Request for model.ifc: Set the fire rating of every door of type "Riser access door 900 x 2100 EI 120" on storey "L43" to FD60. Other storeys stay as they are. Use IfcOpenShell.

First a look at what the model holds.

```python
import ifcopenshell
import ifcopenshell.util.element

model = ifcopenshell.open("model.ifc")
print(model.schema)
storey = next(s for s in model.by_type("IfcBuildingStorey") if s.Name == "L43")
doors = [e for e in ifcopenshell.util.element.get_decomposition(storey) if e.is_a("IfcDoor")]
seen = {}
for e in doors:
    element_type = ifcopenshell.util.element.get_type(e)
    key = (element_type.Name if element_type != e and element_type else None, ifcopenshell.util.element.get_pset(e, "Pset_DoorCommon", "FireRating"))
    seen[key] = seen.get(key, 0) + 1
for (name, value), count in sorted(seen.items(), key=str):
    print(count, "x", name, "|", value)
```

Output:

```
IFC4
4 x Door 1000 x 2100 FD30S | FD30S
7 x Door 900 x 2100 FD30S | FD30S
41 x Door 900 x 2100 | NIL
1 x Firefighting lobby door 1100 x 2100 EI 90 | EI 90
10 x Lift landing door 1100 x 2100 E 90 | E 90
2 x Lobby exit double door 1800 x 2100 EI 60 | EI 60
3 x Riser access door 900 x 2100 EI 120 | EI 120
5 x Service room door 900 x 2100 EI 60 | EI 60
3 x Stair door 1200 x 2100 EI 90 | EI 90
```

```python
import ifcopenshell
import ifcopenshell.api.pset
import ifcopenshell.util.element

model = ifcopenshell.open("model.ifc")

storey = next(s for s in model.by_type("IfcBuildingStorey") if s.Name == "L43")
doors = [e for e in ifcopenshell.util.element.get_decomposition(storey) if e.is_a("IfcDoor")]

count = 0
for e in doors:
    element_type = ifcopenshell.util.element.get_type(e)
    if element_type in (None, e) or element_type.Name != "Riser access door 900 x 2100 EI 120":
        continue
    found = ifcopenshell.util.element.get_pset(e, "Pset_DoorCommon", should_inherit=False)
    if found:
        pset = model.by_id(found["id"])
        if len(ifcopenshell.util.element.get_elements_by_pset(pset)) > 1:
            pset = ifcopenshell.api.pset.unshare_pset(model, products=[e], pset=pset)[0]
    else:
        pset = ifcopenshell.api.pset.add_pset(model, product=e, name="Pset_DoorCommon")
    ifcopenshell.api.pset.edit_pset(model, pset=pset, properties={"FireRating": "FD60"})
    count += 1

print(count, "doors updated")

model.write("model_edited.ifc")
```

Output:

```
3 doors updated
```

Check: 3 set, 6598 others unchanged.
